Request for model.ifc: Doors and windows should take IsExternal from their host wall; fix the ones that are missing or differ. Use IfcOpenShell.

First a look at what the model holds.

```python
import ifcopenshell
import ifcopenshell.util.element

model = ifcopenshell.open("model.ifc")
print(model.schema)
seen = {}
for e in model.by_type("IfcDoor") + model.by_type("IfcWindow"):
    if not e.FillsVoids:
        continue
    host = e.FillsVoids[0].RelatingOpeningElement.VoidsElements[0].RelatingBuildingElement
    own = ifcopenshell.util.element.get_pset(e, f"Pset_{e.is_a()[3:].removesuffix('StandardCase')}Common", "IsExternal")
    wall = ifcopenshell.util.element.get_pset(host, "Pset_WallCommon", "IsExternal")
    seen[e.is_a(), own, wall] = seen.get((e.is_a(), own, wall), 0) + 1
for (cls, own, wall), count in sorted(seen.items(), key=str):
    print(count, cls, "IsExternal:", own, "| host wall:", wall)
```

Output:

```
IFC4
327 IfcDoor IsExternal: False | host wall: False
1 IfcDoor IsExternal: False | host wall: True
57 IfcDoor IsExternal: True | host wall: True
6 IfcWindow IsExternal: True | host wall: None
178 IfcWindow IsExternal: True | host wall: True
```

```python
import ifcopenshell
import ifcopenshell.api.pset
import ifcopenshell.util.element

model = ifcopenshell.open("model.ifc")

count = 0
for ifc_class, pset_name in (("IfcDoor", "Pset_DoorCommon"), ("IfcWindow", "Pset_WindowCommon")):
    for e in model.by_type(ifc_class):
        if not e.FillsVoids:
            continue
        host = e.FillsVoids[0].RelatingOpeningElement.VoidsElements[0].RelatingBuildingElement
        external = ifcopenshell.util.element.get_pset(host, "Pset_WallCommon", "IsExternal")
        if external is None or ifcopenshell.util.element.get_pset(e, pset_name, "IsExternal") == external:
            continue
        pset = ifcopenshell.api.pset.add_pset(model, product=e, name=pset_name)
        ifcopenshell.api.pset.edit_pset(model, pset=pset, properties={"IsExternal": external})
        count += 1

print(count, "updated")

model.write("model_rev.ifc")
```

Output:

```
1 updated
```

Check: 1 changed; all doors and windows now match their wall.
